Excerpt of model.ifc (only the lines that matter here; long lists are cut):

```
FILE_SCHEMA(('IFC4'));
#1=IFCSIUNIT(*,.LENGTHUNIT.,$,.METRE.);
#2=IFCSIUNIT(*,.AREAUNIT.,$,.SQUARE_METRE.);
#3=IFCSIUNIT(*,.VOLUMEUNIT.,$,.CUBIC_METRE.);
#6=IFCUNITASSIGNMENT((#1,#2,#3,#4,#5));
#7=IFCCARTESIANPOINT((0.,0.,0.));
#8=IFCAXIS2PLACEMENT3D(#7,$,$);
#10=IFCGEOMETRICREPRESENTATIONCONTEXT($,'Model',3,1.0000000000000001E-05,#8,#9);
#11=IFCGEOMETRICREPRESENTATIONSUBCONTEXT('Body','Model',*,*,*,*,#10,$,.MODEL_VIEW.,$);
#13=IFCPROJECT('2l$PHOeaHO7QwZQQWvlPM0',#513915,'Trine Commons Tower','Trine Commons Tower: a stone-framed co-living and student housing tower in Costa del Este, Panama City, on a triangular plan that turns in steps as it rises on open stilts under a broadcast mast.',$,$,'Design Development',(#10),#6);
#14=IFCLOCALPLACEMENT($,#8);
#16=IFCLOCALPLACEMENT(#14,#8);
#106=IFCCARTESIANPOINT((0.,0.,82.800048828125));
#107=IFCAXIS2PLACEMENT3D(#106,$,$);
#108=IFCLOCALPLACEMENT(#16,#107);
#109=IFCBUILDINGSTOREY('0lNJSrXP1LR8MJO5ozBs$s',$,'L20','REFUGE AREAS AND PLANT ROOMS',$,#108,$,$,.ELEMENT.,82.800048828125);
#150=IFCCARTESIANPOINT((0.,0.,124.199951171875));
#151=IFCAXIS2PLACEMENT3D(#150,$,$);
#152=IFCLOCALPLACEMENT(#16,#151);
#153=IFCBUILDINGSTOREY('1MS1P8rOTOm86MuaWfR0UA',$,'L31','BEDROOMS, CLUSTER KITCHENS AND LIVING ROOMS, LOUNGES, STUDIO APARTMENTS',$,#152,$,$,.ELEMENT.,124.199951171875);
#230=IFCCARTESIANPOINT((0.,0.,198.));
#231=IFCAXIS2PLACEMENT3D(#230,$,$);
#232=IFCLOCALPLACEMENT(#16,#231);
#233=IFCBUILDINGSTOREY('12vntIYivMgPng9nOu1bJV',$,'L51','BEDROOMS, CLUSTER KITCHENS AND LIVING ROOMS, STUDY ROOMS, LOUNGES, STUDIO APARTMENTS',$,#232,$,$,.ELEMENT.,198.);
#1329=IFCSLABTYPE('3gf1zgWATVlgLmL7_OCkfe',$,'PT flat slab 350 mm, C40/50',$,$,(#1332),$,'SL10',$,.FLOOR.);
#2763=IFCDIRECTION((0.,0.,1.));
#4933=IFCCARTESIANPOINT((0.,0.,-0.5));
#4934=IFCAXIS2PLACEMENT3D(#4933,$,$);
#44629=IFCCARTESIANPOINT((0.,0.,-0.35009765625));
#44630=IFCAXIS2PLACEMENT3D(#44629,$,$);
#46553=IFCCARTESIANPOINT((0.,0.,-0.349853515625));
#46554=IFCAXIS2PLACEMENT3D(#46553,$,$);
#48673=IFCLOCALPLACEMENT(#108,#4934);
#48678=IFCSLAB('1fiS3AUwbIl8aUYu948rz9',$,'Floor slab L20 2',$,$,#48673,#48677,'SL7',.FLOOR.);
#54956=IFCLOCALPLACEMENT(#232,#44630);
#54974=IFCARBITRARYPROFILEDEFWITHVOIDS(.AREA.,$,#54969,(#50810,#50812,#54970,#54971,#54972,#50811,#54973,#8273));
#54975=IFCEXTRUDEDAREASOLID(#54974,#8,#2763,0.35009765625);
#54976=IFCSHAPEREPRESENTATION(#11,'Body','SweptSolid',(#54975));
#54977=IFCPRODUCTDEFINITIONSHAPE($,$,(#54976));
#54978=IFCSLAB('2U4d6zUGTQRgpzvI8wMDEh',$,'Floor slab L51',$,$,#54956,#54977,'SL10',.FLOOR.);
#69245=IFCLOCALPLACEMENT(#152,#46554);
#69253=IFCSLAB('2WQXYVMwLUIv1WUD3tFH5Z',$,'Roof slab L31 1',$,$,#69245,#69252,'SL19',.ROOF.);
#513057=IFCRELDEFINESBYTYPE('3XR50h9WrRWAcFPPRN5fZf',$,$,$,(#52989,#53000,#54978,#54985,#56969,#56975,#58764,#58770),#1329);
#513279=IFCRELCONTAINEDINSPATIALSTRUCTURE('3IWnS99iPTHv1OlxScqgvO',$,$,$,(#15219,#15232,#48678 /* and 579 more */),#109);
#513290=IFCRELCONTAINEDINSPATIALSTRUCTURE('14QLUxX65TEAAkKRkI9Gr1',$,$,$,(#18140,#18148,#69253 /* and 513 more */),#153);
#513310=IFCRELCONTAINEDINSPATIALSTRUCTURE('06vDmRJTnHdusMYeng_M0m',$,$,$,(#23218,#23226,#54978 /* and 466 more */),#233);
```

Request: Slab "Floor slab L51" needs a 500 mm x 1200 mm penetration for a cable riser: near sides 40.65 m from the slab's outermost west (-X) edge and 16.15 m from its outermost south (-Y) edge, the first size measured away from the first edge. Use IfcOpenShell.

```python
import numpy as np
import ifcopenshell
import ifcopenshell.api.feature
import ifcopenshell.api.geometry
import ifcopenshell.api.root
import ifcopenshell.geom
import ifcopenshell.util.placement
import ifcopenshell.util.representation
import ifcopenshell.util.shape
import ifcopenshell.util.unit

model = ifcopenshell.open("model.ifc")
unit_scale = ifcopenshell.util.unit.calculate_unit_scale(model)
settings = ifcopenshell.geom.settings()


def volume(element):
    """Net volume in cubic metres, openings subtracted."""
    shape = ifcopenshell.geom.create_shape(settings, element)
    return ifcopenshell.util.shape.get_volume(shape.geometry)


slab = model.by_guid("2U4d6zUGTQRgpzvI8wMDEh")
before = volume(slab)

# Extent in the slab's own axes, in metres. The edges named are its -X and -Y sides.
slab_shape = ifcopenshell.geom.create_shape(settings, slab)
vertices = ifcopenshell.util.shape.get_vertices(slab_shape.geometry)
x_min, y_min, bottom = vertices.min(axis=0)
top = vertices[:, 2].max()

opening = ifcopenshell.api.root.create_entity(model, ifc_class="IfcOpeningElement", name="Cable riser opening", predefined_type="OPENING")
context = ifcopenshell.util.representation.get_context(model, "Model", "Body", "MODEL_VIEW")
width, depth = 0.5, 1.2
outline = [(0.0, 0.0), (width, 0.0), (width, depth), (0.0, depth), (0.0, 0.0)]
# Overshoot both faces by 50 mm so the cut is clean.
shape = ifcopenshell.api.geometry.add_slab_representation(
    model, context=context, depth=top - bottom + 0.1, polyline=outline
)
ifcopenshell.api.geometry.assign_representation(model, product=opening, representation=shape)

matrix = ifcopenshell.util.placement.get_local_placement(slab.ObjectPlacement)
matrix[:, 3] = matrix @ np.append(np.array([x_min + 40.65, y_min + 16.15, bottom - 0.05]) / unit_scale, 1.0)
ifcopenshell.api.geometry.edit_object_placement(model, product=opening, matrix=matrix, is_si=False)
ifcopenshell.api.feature.add_feature(model, feature=opening, element=slab)

after = volume(slab)

print(f"slab volume {before:.3f} -> {after:.3f} m3")

model.write("model-out.ifc")
```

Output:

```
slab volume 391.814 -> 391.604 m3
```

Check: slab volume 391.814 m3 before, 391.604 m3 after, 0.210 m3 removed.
